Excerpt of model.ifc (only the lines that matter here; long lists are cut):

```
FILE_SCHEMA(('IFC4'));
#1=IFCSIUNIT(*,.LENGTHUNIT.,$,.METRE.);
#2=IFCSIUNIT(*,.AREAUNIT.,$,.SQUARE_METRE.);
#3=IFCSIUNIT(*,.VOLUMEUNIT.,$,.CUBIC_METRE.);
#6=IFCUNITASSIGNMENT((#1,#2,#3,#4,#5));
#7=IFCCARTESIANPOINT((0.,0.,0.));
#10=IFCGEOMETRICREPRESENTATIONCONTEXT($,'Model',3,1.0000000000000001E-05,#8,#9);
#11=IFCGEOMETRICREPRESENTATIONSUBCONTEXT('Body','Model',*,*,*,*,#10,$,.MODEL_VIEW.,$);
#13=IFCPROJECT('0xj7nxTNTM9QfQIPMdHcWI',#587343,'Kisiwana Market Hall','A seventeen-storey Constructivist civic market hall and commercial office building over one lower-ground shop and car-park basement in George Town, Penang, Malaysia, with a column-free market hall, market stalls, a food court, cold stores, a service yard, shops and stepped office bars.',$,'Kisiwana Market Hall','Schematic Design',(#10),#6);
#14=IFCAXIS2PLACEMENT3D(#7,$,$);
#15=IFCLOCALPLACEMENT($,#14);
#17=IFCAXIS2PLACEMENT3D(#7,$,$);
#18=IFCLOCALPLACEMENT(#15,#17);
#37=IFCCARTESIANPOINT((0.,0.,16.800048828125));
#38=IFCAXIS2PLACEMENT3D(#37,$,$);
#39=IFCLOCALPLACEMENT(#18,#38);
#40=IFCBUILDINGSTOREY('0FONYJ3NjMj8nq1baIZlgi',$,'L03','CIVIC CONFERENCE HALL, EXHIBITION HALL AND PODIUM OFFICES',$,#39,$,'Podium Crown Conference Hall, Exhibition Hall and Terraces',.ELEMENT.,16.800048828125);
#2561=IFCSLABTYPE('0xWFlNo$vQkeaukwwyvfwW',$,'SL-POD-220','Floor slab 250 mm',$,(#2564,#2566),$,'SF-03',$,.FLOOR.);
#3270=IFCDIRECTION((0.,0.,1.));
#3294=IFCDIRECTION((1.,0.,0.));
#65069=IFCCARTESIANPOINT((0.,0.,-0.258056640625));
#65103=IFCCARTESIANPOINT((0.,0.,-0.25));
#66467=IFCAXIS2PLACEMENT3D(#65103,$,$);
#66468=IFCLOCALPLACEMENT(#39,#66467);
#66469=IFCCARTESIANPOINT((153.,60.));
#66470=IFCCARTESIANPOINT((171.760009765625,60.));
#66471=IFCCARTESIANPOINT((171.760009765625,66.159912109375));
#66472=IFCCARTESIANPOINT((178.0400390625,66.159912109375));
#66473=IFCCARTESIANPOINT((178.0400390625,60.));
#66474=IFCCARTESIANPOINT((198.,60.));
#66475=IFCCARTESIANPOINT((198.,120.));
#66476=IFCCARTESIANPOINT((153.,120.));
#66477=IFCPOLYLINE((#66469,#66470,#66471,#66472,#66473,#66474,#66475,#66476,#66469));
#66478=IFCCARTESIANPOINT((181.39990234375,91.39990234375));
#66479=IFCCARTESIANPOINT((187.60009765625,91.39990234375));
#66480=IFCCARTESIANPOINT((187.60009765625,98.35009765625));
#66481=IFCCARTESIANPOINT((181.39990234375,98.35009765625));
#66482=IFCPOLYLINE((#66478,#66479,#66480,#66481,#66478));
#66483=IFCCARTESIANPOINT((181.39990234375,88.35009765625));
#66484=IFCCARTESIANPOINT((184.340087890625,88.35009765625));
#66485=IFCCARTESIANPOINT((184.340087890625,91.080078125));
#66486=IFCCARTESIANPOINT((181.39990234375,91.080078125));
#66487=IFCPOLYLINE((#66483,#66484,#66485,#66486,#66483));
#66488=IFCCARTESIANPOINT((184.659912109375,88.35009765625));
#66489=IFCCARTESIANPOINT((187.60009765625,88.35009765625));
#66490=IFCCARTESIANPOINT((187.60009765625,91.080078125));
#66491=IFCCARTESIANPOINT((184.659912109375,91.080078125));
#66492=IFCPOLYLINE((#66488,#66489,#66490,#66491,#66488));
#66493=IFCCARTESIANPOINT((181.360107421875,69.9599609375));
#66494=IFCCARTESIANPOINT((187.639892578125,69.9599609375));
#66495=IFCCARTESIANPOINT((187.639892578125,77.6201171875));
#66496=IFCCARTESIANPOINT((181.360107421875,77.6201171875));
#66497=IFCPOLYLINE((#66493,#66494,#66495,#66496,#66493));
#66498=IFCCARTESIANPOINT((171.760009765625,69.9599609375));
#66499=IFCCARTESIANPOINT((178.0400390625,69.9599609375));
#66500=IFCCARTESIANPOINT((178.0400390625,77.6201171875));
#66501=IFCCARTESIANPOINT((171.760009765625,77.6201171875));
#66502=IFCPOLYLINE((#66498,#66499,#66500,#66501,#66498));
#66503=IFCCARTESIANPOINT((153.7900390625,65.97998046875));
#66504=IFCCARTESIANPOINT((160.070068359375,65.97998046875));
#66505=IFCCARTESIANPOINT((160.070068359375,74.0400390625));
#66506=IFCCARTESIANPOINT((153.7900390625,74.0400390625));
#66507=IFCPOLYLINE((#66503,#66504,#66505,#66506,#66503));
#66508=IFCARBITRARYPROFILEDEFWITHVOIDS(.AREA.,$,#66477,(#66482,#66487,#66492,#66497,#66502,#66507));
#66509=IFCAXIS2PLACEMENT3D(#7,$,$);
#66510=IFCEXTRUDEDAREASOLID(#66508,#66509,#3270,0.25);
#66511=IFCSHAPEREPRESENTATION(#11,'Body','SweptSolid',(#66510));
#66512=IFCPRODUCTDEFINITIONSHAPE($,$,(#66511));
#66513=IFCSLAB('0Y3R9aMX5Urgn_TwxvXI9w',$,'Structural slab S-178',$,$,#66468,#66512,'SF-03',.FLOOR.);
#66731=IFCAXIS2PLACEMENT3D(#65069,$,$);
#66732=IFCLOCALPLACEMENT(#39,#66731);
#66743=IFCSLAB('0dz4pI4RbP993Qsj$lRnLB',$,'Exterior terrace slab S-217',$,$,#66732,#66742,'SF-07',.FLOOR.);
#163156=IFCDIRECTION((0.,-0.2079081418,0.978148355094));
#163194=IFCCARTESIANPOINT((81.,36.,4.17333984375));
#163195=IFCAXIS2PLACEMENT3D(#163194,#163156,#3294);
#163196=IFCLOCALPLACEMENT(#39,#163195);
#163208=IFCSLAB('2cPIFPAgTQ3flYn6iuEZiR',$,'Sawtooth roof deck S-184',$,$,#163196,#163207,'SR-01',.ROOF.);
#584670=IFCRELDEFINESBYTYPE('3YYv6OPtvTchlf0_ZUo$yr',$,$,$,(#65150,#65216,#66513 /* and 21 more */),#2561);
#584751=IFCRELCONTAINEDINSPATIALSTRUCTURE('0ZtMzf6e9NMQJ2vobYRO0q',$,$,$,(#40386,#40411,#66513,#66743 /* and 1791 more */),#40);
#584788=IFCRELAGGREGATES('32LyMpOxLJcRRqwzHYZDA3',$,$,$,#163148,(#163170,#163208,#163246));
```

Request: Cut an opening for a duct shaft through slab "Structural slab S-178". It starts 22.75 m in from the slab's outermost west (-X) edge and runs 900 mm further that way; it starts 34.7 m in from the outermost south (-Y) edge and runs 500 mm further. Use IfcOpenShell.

```python
import numpy as np
import ifcopenshell
import ifcopenshell.api.feature
import ifcopenshell.api.geometry
import ifcopenshell.api.root
import ifcopenshell.geom
import ifcopenshell.util.placement
import ifcopenshell.util.representation
import ifcopenshell.util.shape
import ifcopenshell.util.unit

model = ifcopenshell.open("model.ifc")
unit_scale = ifcopenshell.util.unit.calculate_unit_scale(model)
settings = ifcopenshell.geom.settings()


def volume(element):
    """Net volume in cubic metres, openings subtracted."""
    shape = ifcopenshell.geom.create_shape(settings, element)
    return ifcopenshell.util.shape.get_volume(shape.geometry)


slab = model.by_id(66513)
before = volume(slab)

# Extent in the slab's own axes, in metres. The edges named are its -X and -Y sides.
slab_shape = ifcopenshell.geom.create_shape(settings, slab)
vertices = ifcopenshell.util.shape.get_vertices(slab_shape.geometry)
x_min, y_min, bottom = vertices.min(axis=0)
top = vertices[:, 2].max()

opening = ifcopenshell.api.root.create_entity(model, ifc_class="IfcOpeningElement", name="Duct shaft opening", predefined_type="OPENING")
context = ifcopenshell.util.representation.get_context(model, "Model", "Body", "MODEL_VIEW")
width, depth = 0.9, 0.5
outline = [(0.0, 0.0), (width, 0.0), (width, depth), (0.0, depth), (0.0, 0.0)]
# Overshoot both faces by 50 mm so the cut is clean.
shape = ifcopenshell.api.geometry.add_slab_representation(
    model, context=context, depth=top - bottom + 0.1, polyline=outline
)
ifcopenshell.api.geometry.assign_representation(model, product=opening, representation=shape)

matrix = ifcopenshell.util.placement.get_local_placement(slab.ObjectPlacement)
matrix[:, 3] = matrix @ np.append(np.array([x_min + 22.75, y_min + 34.7, bottom - 0.05]) / unit_scale, 1.0)
ifcopenshell.api.geometry.edit_object_placement(model, product=opening, matrix=matrix, is_si=False)
ifcopenshell.api.feature.add_feature(model, feature=opening, element=slab)

after = volume(slab)

print(f"slab volume {before:.3f} -> {after:.3f} m3")

model.write("model_v2.ifc")
```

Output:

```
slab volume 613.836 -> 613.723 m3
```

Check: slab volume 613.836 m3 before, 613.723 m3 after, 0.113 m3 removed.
